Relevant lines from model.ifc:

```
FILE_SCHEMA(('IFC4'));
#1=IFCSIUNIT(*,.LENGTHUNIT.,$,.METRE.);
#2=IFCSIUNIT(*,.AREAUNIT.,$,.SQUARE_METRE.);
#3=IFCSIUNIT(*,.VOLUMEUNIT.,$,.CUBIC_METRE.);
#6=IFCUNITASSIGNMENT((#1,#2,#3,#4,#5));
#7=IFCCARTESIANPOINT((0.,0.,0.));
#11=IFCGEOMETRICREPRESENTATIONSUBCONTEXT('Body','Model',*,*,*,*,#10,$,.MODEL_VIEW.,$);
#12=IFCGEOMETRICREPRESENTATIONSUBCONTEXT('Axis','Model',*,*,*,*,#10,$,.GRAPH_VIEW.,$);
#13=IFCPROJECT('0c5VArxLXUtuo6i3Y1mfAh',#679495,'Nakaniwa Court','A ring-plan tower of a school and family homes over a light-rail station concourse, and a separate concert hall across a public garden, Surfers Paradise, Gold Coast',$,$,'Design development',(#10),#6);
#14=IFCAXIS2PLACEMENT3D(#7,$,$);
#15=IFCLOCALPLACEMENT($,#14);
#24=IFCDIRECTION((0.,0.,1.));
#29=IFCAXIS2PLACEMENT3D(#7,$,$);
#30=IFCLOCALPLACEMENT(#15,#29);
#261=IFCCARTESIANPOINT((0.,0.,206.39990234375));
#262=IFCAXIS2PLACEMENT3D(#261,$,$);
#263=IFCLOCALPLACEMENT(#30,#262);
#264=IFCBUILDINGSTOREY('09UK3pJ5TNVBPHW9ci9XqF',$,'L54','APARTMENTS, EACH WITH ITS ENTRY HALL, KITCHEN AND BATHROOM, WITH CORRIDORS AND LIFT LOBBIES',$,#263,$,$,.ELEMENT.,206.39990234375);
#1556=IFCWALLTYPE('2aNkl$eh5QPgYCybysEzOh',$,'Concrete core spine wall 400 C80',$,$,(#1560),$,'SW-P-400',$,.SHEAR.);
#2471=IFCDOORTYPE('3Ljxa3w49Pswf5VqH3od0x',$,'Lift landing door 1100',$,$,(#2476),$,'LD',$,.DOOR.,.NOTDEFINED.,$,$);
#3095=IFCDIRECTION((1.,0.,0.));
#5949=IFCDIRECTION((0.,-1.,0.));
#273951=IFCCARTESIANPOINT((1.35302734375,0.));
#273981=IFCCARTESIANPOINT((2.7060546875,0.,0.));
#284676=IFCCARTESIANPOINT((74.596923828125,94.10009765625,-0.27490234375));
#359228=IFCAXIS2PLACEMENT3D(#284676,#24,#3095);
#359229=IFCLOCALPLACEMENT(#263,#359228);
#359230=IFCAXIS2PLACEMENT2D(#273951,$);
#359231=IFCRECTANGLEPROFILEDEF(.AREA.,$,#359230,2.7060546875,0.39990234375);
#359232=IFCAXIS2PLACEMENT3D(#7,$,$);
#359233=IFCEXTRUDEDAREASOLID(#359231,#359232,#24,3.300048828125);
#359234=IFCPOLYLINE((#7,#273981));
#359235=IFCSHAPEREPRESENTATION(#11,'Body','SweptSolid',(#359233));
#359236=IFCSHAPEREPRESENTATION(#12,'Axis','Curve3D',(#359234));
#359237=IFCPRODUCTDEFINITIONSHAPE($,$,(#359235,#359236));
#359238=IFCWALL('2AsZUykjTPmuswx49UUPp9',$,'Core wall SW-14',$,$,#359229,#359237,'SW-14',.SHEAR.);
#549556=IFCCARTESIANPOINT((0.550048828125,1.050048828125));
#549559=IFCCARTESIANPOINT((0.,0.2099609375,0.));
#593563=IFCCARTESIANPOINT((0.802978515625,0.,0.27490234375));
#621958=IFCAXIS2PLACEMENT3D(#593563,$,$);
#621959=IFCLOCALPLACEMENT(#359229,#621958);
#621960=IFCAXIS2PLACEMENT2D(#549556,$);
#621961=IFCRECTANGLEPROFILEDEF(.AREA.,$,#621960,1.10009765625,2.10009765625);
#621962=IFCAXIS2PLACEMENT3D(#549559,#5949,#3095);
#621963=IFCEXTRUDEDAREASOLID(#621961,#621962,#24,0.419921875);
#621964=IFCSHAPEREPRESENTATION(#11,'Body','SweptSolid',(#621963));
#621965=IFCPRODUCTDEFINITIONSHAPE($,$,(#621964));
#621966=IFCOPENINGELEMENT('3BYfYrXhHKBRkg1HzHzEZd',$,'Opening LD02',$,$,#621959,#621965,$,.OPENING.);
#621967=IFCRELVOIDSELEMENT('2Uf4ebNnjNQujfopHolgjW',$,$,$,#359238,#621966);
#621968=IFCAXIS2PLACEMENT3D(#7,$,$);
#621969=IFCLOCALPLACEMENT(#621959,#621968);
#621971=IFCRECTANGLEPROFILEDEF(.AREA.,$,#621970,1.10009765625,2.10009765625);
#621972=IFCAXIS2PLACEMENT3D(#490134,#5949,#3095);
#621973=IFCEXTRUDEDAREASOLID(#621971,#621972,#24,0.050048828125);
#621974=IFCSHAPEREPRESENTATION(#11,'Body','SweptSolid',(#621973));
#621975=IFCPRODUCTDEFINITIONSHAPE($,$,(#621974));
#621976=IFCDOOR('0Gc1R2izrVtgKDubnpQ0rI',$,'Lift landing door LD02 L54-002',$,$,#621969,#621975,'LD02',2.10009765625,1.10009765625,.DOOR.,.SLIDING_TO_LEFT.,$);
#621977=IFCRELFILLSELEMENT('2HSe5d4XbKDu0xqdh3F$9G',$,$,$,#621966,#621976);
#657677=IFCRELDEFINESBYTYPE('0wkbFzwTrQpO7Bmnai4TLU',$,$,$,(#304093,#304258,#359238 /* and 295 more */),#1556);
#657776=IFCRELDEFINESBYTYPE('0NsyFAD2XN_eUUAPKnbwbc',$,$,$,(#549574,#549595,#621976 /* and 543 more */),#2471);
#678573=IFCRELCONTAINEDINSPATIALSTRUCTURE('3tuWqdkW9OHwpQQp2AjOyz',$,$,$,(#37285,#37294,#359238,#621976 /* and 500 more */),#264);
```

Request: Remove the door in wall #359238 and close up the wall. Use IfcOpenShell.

```python
import ifcopenshell
import ifcopenshell.api.feature
import ifcopenshell.api.root
import ifcopenshell.geom
import ifcopenshell.util.shape

model = ifcopenshell.open("model.ifc")
settings = ifcopenshell.geom.settings()


def volume(element):
    """Net volume in cubic metres, openings subtracted."""
    shape = ifcopenshell.geom.create_shape(settings, element)
    return ifcopenshell.util.shape.get_volume(shape.geometry)


door = model.by_guid("0Gc1R2izrVtgKDubnpQ0rI")
opening = door.FillsVoids[0].RelatingOpeningElement
wall = opening.VoidsElements[0].RelatingBuildingElement
before = volume(wall)

ifcopenshell.api.root.remove_product(model, product=door)
ifcopenshell.api.feature.remove_feature(model, feature=opening)

after = volume(wall)

print(f"wall volume {before:.3f} -> {after:.3f} m3")

model.write("model_rev.ifc")
```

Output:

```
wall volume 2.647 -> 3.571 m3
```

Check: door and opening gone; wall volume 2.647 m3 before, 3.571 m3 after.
